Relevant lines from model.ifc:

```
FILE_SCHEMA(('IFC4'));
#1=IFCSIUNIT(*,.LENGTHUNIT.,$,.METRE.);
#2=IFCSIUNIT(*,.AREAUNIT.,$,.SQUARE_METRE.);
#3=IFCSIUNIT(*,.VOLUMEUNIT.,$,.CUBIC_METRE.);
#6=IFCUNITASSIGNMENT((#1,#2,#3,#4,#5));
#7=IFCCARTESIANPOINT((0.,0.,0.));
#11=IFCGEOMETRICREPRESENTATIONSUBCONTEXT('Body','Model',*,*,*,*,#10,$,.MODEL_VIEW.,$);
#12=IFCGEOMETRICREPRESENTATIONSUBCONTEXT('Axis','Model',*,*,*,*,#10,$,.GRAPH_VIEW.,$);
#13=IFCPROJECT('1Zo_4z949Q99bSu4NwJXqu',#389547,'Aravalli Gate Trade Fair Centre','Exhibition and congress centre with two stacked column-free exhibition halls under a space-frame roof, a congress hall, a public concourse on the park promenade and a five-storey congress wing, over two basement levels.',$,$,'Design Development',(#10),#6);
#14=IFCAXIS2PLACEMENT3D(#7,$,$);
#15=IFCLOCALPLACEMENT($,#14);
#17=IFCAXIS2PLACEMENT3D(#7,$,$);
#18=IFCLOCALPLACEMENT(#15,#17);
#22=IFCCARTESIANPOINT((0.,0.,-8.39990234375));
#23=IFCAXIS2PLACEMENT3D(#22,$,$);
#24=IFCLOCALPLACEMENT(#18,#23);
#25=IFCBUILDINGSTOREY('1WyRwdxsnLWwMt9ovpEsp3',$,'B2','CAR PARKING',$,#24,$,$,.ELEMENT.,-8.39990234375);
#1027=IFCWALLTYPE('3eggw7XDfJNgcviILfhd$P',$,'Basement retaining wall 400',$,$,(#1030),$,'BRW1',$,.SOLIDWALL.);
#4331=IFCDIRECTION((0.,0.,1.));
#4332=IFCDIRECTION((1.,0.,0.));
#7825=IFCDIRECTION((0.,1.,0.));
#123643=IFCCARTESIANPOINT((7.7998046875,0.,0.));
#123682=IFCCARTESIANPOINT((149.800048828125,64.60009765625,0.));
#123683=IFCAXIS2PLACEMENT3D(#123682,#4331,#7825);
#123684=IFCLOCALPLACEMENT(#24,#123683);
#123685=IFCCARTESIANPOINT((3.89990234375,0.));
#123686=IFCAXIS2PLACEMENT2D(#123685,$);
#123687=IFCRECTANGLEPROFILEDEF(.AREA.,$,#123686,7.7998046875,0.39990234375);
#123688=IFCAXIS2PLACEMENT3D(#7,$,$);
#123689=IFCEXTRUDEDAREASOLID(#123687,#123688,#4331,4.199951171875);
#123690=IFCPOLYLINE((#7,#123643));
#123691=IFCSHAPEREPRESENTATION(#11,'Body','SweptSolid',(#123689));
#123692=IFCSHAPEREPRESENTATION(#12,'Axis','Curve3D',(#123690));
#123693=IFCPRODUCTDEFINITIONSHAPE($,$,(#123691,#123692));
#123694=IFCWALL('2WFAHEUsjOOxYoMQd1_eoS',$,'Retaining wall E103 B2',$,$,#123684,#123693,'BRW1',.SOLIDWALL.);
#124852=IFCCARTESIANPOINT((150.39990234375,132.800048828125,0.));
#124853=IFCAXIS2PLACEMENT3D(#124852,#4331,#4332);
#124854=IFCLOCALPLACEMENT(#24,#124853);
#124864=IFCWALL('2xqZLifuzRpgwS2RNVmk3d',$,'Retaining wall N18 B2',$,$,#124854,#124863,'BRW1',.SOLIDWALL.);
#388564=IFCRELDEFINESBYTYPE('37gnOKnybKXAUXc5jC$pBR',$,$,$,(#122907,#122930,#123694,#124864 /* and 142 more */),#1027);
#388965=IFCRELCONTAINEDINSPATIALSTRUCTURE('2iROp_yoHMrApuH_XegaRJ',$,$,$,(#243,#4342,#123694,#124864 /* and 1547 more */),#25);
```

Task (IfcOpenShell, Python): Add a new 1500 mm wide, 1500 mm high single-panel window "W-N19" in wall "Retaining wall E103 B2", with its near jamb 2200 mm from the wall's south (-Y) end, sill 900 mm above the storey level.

```python
import numpy as np
import ifcopenshell
import ifcopenshell.api.feature
import ifcopenshell.api.geometry
import ifcopenshell.api.root
import ifcopenshell.api.spatial
import ifcopenshell.geom
import ifcopenshell.util.element
import ifcopenshell.util.placement
import ifcopenshell.util.representation
import ifcopenshell.util.shape
import ifcopenshell.util.unit

model = ifcopenshell.open("model.ifc")
unit_scale = ifcopenshell.util.unit.calculate_unit_scale(model)
settings = ifcopenshell.geom.settings()


def volume(element):
    """Net volume in cubic metres, openings subtracted."""
    shape = ifcopenshell.geom.create_shape(settings, element)
    return ifcopenshell.util.shape.get_volume(shape.geometry)


wall = model.by_guid("2WFAHEUsjOOxYoMQd1_eoS")
storey = ifcopenshell.util.element.get_container(wall, ifc_class="IfcBuildingStorey")
context = ifcopenshell.util.representation.get_context(model, "Model", "Body", "MODEL_VIEW")
before = volume(wall)

width, height, from_end, sill = 1.5, 1.5, 2.2, 0.9  # metres

# The wall runs along its own X axis, and the end named is its -X end.
wall_shape = ifcopenshell.geom.create_shape(settings, wall)
x, y, z = ifcopenshell.util.shape.get_vertices(wall_shape.geometry).T
start = x.min() + from_end
face, thickness = float(y.min()), float(y.max() - y.min())
wall_matrix = ifcopenshell.util.placement.get_local_placement(wall.ObjectPlacement)
level = ifcopenshell.util.placement.get_local_placement(storey.ObjectPlacement)[2, 3]


def in_wall(x, y):
    """Placement at x, y metres in the wall's axes, at sill height."""
    matrix = wall_matrix.copy()
    matrix[:, 3] = wall_matrix @ np.array([x / unit_scale, y / unit_scale, 0.0, 1.0])
    matrix[2, 3] = level + sill / unit_scale
    return matrix


# Opening: a box that overshoots both wall faces by 50 mm.
opening = ifcopenshell.api.root.create_entity(model, ifc_class="IfcOpeningElement", predefined_type="OPENING")
box = ifcopenshell.api.geometry.add_wall_representation(
    model, context=context, length=width, height=height, thickness=thickness + 0.1
)
ifcopenshell.api.geometry.assign_representation(model, product=opening, representation=box)
ifcopenshell.api.geometry.edit_object_placement(model, product=opening, matrix=in_wall(start, face - 0.05), is_si=False)
ifcopenshell.api.feature.add_feature(model, feature=opening, element=wall)

window = ifcopenshell.api.root.create_entity(model, ifc_class="IfcWindow", name="W-N19", predefined_type="WINDOW")
window.OverallWidth, window.OverallHeight = width / unit_scale, height / unit_scale
window.PartitioningType = "SINGLE_PANEL"
body = ifcopenshell.api.geometry.add_window_representation(
    model,
    context=context,
    overall_width=window.OverallWidth,
    overall_height=window.OverallHeight,
    partition_type="SINGLE_PANEL",
)
ifcopenshell.api.geometry.assign_representation(model, product=window, representation=body)
ifcopenshell.api.spatial.assign_container(model, products=[window], relating_structure=storey)
ifcopenshell.api.feature.add_filling(model, opening=opening, element=window)

# Centre the window in the wall's thickness.
ifcopenshell.api.geometry.edit_object_placement(model, product=window, matrix=in_wall(start, face), is_si=False)
window_shape = ifcopenshell.geom.create_shape(settings, window)
depth = ifcopenshell.util.shape.get_vertices(window_shape.geometry)[:, 1]
offset = face + thickness / 2 - (depth.min() + depth.max()) / 2
ifcopenshell.api.geometry.edit_object_placement(model, product=window, matrix=in_wall(start, offset), is_si=False)

after = volume(wall)

print(f"wall volume {before:.3f} -> {after:.3f} m3")

model.write("model_v2.ifc")
```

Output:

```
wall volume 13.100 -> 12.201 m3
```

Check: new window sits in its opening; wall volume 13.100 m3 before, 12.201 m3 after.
